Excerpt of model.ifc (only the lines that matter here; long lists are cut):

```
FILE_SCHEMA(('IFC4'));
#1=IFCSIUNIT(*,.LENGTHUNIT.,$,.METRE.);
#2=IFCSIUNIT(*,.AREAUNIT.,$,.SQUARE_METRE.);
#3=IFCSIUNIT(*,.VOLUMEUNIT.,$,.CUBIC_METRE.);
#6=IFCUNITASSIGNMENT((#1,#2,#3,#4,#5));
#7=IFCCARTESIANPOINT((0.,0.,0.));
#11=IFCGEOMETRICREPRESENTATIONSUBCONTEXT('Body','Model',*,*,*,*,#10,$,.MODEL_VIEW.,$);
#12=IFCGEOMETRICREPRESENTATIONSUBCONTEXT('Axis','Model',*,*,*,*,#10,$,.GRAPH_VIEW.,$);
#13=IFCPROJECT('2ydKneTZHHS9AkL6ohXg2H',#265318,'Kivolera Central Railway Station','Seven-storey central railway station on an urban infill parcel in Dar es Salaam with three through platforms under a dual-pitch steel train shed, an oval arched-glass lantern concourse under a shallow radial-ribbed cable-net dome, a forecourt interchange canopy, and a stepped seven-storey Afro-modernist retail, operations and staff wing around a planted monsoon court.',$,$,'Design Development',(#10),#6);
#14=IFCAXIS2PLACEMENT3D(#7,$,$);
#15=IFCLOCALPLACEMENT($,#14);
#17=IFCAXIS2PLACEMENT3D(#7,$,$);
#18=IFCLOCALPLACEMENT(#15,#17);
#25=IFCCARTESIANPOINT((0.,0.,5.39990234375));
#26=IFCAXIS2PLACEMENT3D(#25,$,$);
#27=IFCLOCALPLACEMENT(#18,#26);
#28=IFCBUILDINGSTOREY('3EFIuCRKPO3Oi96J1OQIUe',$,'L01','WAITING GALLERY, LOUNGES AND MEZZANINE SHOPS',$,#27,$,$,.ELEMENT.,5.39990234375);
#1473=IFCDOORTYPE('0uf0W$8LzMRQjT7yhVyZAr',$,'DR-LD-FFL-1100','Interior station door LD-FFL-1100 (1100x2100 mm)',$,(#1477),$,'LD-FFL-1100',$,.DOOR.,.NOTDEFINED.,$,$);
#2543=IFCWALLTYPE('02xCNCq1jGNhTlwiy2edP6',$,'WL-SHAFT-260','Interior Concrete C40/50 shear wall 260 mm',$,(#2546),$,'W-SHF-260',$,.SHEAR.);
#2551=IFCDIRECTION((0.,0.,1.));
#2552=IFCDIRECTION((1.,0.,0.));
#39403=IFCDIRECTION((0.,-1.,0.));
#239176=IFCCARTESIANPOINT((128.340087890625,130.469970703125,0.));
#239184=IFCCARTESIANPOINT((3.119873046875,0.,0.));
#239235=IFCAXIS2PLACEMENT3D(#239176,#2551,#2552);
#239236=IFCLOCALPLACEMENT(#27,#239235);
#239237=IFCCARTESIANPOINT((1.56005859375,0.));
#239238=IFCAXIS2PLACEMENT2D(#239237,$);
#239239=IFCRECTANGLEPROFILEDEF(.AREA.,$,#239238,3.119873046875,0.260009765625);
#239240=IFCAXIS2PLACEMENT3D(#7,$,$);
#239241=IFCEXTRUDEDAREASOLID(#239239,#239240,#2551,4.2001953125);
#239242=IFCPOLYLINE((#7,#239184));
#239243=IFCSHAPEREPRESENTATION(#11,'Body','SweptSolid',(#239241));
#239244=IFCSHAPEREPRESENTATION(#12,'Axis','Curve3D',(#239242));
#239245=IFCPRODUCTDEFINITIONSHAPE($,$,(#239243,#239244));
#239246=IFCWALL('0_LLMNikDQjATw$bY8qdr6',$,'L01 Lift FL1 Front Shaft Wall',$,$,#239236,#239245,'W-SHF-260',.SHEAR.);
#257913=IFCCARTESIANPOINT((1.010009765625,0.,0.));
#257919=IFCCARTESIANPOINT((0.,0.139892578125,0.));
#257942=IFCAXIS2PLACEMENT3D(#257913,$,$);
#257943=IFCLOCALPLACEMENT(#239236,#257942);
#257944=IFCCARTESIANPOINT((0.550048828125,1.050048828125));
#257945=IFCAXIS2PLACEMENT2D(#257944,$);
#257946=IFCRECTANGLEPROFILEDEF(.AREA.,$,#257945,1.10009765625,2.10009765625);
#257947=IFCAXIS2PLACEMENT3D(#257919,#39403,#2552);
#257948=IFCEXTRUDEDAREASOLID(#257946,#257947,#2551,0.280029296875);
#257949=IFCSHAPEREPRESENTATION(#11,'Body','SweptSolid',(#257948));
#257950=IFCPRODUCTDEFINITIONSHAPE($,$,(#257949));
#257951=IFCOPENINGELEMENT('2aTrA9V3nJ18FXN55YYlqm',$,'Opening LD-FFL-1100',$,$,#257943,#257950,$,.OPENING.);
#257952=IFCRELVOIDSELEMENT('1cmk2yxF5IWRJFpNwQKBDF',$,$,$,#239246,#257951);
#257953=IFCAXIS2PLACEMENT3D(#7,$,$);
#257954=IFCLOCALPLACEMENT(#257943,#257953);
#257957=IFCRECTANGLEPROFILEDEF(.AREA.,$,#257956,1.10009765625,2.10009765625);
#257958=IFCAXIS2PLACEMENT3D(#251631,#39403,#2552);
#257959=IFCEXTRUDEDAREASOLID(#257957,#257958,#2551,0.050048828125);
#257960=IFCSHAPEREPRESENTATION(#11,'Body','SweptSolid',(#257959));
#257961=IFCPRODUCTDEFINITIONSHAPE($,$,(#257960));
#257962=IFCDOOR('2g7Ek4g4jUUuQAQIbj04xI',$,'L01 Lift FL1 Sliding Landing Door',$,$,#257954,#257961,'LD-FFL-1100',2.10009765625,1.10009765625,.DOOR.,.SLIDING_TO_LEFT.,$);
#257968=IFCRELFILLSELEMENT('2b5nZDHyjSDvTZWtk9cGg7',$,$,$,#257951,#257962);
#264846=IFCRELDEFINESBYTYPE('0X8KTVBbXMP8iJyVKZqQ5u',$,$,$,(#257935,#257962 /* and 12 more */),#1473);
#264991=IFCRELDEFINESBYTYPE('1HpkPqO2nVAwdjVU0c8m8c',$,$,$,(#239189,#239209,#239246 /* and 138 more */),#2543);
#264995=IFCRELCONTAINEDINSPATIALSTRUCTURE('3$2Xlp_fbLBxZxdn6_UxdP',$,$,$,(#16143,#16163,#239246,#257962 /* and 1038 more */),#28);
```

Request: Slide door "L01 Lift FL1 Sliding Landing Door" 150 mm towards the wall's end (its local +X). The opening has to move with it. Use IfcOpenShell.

```python
import ifcopenshell
import ifcopenshell.api.geometry
import ifcopenshell.util.placement
import ifcopenshell.util.unit

model = ifcopenshell.open("model.ifc")
unit_scale = ifcopenshell.util.unit.calculate_unit_scale(model)

door = model.by_guid("2g7Ek4g4jUUuQAQIbj04xI")
opening = door.FillsVoids[0].RelatingOpeningElement
wall = opening.VoidsElements[0].RelatingBuildingElement

wall_matrix = ifcopenshell.util.placement.get_local_placement(wall.ObjectPlacement)
shift = wall_matrix[:3, 0] * 0.15 / unit_scale
before = ifcopenshell.util.placement.get_local_placement(door.ObjectPlacement)[:3, 3].copy()

# The door is placed relative to its opening, so it follows when the opening moves.
matrix = ifcopenshell.util.placement.get_local_placement(opening.ObjectPlacement)
matrix[:3, 3] += shift
ifcopenshell.api.geometry.edit_object_placement(
    model, product=opening, matrix=matrix, is_si=False, should_transform_children=True
)

after = ifcopenshell.util.placement.get_local_placement(door.ObjectPlacement)[:3, 3]
print("door moved by", (after - before).round(3) + 0.0)

model.write("model-out.ifc")
```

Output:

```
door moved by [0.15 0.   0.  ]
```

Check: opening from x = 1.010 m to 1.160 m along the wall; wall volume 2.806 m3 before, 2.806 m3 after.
